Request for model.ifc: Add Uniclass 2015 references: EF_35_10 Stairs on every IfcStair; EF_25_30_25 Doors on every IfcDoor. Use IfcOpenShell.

First a look at what the model holds.

```python
import ifcopenshell

model = ifcopenshell.open("model.ifc")
print(model.schema)
print("classifications:", [c.Name for c in model.by_type("IfcClassification")])
for ifc_class in ("IfcDoor", "IfcRoof", "IfcStair", "IfcWall", "IfcWindow"):
    print(ifc_class, len(model.by_type(ifc_class)))
```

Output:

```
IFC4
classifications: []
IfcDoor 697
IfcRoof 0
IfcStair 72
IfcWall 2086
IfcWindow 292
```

```python
import ifcopenshell
import ifcopenshell.api.classification

model = ifcopenshell.open("model.ifc")

system = ifcopenshell.api.classification.add_classification(model, classification="Uniclass 2015")

codes = {
    "IfcStair": ("EF_35_10", "Stairs"),
    "IfcDoor": ("EF_25_30_25", "Doors"),
}
for ifc_class, (code, name) in codes.items():
    products = model.by_type(ifc_class)
    ifcopenshell.api.classification.add_reference(
        model, products=products, classification=system, identification=code, name=name
    )
    print(code, len(products))

model.write("model_v2.ifc")
```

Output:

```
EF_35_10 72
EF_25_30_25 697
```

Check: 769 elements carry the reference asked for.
